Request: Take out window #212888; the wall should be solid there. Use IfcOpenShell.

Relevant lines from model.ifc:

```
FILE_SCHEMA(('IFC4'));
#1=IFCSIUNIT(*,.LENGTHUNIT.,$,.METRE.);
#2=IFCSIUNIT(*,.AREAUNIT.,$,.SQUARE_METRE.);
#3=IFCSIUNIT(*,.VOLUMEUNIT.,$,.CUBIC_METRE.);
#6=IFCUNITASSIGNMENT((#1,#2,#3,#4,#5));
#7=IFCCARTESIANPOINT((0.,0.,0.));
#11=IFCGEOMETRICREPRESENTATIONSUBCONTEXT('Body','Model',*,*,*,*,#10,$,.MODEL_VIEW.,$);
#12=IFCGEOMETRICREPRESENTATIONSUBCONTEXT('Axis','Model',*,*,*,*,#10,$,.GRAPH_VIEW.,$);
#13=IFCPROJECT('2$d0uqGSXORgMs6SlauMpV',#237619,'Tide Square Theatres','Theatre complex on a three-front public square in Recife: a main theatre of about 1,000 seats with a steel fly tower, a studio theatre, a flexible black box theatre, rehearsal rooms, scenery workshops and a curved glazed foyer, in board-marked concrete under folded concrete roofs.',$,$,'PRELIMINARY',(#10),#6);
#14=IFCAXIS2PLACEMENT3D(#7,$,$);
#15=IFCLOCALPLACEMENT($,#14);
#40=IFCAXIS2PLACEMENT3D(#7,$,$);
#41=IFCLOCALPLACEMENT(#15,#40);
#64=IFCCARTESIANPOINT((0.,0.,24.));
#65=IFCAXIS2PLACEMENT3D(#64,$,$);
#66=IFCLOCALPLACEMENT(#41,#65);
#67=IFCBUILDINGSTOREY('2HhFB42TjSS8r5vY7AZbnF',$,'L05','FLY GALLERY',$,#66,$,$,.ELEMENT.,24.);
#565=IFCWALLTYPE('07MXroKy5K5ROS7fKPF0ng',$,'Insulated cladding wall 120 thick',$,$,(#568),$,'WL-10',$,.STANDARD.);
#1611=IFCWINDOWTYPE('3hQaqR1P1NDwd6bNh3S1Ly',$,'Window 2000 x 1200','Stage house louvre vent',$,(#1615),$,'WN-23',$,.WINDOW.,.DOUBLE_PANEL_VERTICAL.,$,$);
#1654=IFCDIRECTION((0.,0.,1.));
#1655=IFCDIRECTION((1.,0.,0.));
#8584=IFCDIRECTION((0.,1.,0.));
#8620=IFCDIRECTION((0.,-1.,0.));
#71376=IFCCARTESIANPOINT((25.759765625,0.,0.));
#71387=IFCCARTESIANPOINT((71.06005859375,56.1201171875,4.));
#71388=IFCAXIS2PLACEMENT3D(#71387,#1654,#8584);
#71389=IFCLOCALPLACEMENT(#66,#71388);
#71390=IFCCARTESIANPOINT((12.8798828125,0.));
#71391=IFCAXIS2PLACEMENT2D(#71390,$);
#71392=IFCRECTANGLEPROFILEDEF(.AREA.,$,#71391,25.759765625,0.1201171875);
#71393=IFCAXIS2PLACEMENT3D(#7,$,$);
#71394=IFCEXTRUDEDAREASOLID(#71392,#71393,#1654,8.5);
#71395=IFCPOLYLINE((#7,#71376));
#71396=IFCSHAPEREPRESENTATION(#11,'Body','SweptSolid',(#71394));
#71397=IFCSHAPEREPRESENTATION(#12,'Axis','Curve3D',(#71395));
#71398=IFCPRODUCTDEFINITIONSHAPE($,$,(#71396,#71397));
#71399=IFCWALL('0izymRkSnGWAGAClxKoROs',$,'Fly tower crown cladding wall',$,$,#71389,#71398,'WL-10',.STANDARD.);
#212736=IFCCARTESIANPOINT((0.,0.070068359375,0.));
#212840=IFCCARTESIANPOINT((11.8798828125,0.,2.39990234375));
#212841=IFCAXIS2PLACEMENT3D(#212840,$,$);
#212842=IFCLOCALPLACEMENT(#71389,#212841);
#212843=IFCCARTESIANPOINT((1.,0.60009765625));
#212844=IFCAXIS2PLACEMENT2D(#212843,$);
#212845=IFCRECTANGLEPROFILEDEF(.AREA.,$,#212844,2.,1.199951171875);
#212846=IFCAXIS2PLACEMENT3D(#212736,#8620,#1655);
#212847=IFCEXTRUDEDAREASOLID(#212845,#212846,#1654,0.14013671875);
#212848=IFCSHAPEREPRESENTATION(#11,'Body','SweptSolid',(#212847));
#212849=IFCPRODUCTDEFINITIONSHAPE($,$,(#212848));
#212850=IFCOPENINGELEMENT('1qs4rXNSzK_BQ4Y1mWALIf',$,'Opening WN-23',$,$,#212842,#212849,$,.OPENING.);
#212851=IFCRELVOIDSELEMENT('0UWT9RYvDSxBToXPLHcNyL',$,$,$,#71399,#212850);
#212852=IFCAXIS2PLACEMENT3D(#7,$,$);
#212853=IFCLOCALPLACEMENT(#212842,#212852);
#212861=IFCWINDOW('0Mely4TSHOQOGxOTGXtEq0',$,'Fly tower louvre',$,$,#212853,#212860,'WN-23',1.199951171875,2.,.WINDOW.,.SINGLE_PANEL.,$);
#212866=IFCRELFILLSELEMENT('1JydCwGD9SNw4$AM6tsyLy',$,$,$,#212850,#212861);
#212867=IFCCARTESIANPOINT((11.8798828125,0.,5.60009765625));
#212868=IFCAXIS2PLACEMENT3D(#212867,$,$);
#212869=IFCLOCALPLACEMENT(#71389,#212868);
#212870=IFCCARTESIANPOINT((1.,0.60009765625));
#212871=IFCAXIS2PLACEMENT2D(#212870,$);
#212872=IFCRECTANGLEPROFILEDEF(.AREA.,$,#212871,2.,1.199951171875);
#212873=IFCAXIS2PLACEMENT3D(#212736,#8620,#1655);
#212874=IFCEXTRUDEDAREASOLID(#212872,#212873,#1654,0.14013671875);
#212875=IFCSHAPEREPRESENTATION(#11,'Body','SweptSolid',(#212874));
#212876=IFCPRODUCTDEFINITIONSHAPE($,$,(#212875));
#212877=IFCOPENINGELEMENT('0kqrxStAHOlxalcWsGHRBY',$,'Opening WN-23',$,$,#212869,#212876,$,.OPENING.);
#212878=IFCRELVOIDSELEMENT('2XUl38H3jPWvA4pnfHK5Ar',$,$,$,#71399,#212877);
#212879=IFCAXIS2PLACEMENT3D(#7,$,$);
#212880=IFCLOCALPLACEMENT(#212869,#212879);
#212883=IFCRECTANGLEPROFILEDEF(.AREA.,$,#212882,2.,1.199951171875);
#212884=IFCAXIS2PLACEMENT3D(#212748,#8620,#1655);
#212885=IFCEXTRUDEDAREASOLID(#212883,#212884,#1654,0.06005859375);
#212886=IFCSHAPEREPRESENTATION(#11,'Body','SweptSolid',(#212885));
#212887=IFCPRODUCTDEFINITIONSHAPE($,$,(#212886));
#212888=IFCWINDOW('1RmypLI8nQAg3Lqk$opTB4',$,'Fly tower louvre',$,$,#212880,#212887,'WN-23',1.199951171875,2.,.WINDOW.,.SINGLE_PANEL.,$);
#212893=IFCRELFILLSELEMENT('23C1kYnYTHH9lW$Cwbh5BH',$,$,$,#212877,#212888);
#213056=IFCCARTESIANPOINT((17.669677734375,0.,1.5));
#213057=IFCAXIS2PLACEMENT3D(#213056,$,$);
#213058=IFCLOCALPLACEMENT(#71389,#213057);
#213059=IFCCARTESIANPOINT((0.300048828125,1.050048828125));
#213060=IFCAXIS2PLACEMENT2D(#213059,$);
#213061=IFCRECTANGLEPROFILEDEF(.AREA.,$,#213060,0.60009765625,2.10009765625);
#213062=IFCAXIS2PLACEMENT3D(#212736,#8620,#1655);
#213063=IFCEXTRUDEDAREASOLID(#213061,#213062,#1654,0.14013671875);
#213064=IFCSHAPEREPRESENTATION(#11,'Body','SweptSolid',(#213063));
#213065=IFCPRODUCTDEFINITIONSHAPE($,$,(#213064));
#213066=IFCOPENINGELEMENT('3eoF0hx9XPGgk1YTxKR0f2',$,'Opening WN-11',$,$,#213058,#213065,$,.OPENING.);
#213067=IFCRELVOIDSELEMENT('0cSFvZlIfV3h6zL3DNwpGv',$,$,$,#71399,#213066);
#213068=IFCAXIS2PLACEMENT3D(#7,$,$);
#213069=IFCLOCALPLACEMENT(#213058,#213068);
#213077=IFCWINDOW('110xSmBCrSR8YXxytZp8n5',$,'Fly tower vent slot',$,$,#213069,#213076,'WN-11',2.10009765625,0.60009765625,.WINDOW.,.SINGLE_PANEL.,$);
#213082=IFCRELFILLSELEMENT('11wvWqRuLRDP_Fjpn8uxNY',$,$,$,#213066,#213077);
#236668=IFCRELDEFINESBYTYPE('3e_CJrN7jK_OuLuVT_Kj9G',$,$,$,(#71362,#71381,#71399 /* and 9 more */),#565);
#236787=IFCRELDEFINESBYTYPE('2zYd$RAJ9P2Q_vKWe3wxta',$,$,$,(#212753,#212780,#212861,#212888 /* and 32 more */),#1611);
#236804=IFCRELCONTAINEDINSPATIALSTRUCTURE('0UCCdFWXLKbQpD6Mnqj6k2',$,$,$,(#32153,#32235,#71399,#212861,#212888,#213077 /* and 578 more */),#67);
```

```python
import ifcopenshell
import ifcopenshell.api.feature
import ifcopenshell.api.root
import ifcopenshell.geom
import ifcopenshell.util.shape

model = ifcopenshell.open("model.ifc")
settings = ifcopenshell.geom.settings()


def volume(element):
    """Net volume in cubic metres, openings subtracted."""
    shape = ifcopenshell.geom.create_shape(settings, element)
    return ifcopenshell.util.shape.get_volume(shape.geometry)


window = model.by_id(212888)
opening = window.FillsVoids[0].RelatingOpeningElement
wall = opening.VoidsElements[0].RelatingBuildingElement
before = volume(wall)

ifcopenshell.api.root.remove_product(model, product=window)
ifcopenshell.api.feature.remove_feature(model, feature=opening)

after = volume(wall)

print(f"wall volume {before:.3f} -> {after:.3f} m3")

model.write("model_rev.ifc")
```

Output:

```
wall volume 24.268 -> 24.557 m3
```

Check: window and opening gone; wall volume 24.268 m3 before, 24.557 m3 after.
